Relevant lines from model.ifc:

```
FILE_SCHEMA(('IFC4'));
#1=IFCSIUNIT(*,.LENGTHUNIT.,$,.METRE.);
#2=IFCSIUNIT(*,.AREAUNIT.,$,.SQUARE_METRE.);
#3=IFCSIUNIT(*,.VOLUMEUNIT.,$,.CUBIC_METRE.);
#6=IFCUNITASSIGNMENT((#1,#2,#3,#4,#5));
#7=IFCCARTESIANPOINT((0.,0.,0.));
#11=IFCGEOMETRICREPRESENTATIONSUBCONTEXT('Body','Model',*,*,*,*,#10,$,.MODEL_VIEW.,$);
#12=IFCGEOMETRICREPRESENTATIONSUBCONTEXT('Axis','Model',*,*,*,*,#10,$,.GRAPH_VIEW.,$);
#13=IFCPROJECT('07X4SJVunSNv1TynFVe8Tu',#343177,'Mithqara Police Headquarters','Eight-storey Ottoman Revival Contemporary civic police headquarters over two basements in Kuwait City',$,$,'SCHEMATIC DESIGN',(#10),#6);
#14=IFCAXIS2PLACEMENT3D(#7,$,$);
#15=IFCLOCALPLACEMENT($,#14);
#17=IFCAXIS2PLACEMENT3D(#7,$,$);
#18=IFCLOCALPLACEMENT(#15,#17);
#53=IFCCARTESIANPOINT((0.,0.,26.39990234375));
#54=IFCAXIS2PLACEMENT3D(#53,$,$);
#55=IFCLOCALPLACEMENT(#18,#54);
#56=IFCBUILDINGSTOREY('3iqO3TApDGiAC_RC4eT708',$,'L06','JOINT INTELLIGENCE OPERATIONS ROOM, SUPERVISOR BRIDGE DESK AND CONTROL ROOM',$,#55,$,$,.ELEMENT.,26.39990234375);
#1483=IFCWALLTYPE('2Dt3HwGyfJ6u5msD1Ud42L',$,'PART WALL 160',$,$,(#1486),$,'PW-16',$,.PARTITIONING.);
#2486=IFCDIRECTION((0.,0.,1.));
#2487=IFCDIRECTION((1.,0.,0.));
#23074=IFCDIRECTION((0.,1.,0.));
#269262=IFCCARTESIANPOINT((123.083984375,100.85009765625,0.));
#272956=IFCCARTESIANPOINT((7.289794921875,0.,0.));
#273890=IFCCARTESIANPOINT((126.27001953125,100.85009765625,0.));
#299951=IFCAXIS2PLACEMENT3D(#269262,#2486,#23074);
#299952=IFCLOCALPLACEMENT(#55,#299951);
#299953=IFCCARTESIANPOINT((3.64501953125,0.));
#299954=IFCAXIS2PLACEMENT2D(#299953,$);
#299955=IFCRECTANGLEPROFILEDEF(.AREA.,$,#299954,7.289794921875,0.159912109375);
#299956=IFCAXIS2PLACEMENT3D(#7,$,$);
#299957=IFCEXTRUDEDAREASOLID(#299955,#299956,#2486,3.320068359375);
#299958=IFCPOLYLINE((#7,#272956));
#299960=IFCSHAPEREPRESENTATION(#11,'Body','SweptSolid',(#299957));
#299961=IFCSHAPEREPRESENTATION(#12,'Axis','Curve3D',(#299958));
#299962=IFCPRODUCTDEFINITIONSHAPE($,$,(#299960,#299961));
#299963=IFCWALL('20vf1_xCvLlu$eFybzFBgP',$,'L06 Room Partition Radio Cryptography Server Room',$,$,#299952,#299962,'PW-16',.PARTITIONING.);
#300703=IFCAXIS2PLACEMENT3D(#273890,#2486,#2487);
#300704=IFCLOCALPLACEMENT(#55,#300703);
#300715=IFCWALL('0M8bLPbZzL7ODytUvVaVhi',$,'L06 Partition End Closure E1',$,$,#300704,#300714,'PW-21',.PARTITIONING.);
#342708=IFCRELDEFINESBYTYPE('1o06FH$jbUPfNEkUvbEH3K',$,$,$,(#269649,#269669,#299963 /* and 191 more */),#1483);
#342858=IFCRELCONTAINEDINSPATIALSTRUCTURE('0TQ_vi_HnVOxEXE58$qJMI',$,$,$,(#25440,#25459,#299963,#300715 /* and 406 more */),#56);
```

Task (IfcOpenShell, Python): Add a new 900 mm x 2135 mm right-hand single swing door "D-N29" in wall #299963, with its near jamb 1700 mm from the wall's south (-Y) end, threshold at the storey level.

```python
import numpy as np
import ifcopenshell
import ifcopenshell.api.feature
import ifcopenshell.api.geometry
import ifcopenshell.api.root
import ifcopenshell.api.spatial
import ifcopenshell.geom
import ifcopenshell.util.element
import ifcopenshell.util.placement
import ifcopenshell.util.representation
import ifcopenshell.util.shape
import ifcopenshell.util.unit

model = ifcopenshell.open("model.ifc")
unit_scale = ifcopenshell.util.unit.calculate_unit_scale(model)
settings = ifcopenshell.geom.settings()


def volume(element):
    """Net volume in cubic metres, openings subtracted."""
    shape = ifcopenshell.geom.create_shape(settings, element)
    return ifcopenshell.util.shape.get_volume(shape.geometry)


wall = model.by_guid("20vf1_xCvLlu$eFybzFBgP")
storey = ifcopenshell.util.element.get_container(wall, ifc_class="IfcBuildingStorey")
context = ifcopenshell.util.representation.get_context(model, "Model", "Body", "MODEL_VIEW")
before = volume(wall)

width, height, from_end, sill = 0.9, 2.135, 1.7, 0.0  # metres

# The wall runs along its own X axis, and the end named is its -X end.
wall_shape = ifcopenshell.geom.create_shape(settings, wall)
x, y, z = ifcopenshell.util.shape.get_vertices(wall_shape.geometry).T
start = x.min() + from_end
face, thickness = float(y.min()), float(y.max() - y.min())
wall_matrix = ifcopenshell.util.placement.get_local_placement(wall.ObjectPlacement)
level = ifcopenshell.util.placement.get_local_placement(storey.ObjectPlacement)[2, 3]


def in_wall(x, y):
    """Placement at x, y metres in the wall's axes, at sill height."""
    matrix = wall_matrix.copy()
    matrix[:, 3] = wall_matrix @ np.array([x / unit_scale, y / unit_scale, 0.0, 1.0])
    matrix[2, 3] = level + sill / unit_scale
    return matrix


# Opening: a box that overshoots both wall faces by 50 mm.
opening = ifcopenshell.api.root.create_entity(model, ifc_class="IfcOpeningElement", predefined_type="OPENING")
box = ifcopenshell.api.geometry.add_wall_representation(
    model, context=context, length=width, height=height, thickness=thickness + 0.1
)
ifcopenshell.api.geometry.assign_representation(model, product=opening, representation=box)
ifcopenshell.api.geometry.edit_object_placement(model, product=opening, matrix=in_wall(start, face - 0.05), is_si=False)
ifcopenshell.api.feature.add_feature(model, feature=opening, element=wall)

door = ifcopenshell.api.root.create_entity(model, ifc_class="IfcDoor", name="D-N29", predefined_type="DOOR")
door.OverallWidth, door.OverallHeight = width / unit_scale, height / unit_scale
door.OperationType = "SINGLE_SWING_RIGHT"
body = ifcopenshell.api.geometry.add_door_representation(
    model,
    context=context,
    overall_width=door.OverallWidth,
    overall_height=door.OverallHeight,
    operation_type="SINGLE_SWING_RIGHT",
    lining_properties={"LiningDepth": thickness / unit_scale, "ThresholdDepth": thickness / unit_scale},
)
ifcopenshell.api.geometry.assign_representation(model, product=door, representation=body)
ifcopenshell.api.spatial.assign_container(model, products=[door], relating_structure=storey)
ifcopenshell.api.feature.add_filling(model, opening=opening, element=door)

# The lining spans the wall, so the door starts at the wall face.
ifcopenshell.api.geometry.edit_object_placement(model, product=door, matrix=in_wall(start, face), is_si=False)

after = volume(wall)

print(f"wall volume {before:.3f} -> {after:.3f} m3")

model.write("model_edited.ifc")
```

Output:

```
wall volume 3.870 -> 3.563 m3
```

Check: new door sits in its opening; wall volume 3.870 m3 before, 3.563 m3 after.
